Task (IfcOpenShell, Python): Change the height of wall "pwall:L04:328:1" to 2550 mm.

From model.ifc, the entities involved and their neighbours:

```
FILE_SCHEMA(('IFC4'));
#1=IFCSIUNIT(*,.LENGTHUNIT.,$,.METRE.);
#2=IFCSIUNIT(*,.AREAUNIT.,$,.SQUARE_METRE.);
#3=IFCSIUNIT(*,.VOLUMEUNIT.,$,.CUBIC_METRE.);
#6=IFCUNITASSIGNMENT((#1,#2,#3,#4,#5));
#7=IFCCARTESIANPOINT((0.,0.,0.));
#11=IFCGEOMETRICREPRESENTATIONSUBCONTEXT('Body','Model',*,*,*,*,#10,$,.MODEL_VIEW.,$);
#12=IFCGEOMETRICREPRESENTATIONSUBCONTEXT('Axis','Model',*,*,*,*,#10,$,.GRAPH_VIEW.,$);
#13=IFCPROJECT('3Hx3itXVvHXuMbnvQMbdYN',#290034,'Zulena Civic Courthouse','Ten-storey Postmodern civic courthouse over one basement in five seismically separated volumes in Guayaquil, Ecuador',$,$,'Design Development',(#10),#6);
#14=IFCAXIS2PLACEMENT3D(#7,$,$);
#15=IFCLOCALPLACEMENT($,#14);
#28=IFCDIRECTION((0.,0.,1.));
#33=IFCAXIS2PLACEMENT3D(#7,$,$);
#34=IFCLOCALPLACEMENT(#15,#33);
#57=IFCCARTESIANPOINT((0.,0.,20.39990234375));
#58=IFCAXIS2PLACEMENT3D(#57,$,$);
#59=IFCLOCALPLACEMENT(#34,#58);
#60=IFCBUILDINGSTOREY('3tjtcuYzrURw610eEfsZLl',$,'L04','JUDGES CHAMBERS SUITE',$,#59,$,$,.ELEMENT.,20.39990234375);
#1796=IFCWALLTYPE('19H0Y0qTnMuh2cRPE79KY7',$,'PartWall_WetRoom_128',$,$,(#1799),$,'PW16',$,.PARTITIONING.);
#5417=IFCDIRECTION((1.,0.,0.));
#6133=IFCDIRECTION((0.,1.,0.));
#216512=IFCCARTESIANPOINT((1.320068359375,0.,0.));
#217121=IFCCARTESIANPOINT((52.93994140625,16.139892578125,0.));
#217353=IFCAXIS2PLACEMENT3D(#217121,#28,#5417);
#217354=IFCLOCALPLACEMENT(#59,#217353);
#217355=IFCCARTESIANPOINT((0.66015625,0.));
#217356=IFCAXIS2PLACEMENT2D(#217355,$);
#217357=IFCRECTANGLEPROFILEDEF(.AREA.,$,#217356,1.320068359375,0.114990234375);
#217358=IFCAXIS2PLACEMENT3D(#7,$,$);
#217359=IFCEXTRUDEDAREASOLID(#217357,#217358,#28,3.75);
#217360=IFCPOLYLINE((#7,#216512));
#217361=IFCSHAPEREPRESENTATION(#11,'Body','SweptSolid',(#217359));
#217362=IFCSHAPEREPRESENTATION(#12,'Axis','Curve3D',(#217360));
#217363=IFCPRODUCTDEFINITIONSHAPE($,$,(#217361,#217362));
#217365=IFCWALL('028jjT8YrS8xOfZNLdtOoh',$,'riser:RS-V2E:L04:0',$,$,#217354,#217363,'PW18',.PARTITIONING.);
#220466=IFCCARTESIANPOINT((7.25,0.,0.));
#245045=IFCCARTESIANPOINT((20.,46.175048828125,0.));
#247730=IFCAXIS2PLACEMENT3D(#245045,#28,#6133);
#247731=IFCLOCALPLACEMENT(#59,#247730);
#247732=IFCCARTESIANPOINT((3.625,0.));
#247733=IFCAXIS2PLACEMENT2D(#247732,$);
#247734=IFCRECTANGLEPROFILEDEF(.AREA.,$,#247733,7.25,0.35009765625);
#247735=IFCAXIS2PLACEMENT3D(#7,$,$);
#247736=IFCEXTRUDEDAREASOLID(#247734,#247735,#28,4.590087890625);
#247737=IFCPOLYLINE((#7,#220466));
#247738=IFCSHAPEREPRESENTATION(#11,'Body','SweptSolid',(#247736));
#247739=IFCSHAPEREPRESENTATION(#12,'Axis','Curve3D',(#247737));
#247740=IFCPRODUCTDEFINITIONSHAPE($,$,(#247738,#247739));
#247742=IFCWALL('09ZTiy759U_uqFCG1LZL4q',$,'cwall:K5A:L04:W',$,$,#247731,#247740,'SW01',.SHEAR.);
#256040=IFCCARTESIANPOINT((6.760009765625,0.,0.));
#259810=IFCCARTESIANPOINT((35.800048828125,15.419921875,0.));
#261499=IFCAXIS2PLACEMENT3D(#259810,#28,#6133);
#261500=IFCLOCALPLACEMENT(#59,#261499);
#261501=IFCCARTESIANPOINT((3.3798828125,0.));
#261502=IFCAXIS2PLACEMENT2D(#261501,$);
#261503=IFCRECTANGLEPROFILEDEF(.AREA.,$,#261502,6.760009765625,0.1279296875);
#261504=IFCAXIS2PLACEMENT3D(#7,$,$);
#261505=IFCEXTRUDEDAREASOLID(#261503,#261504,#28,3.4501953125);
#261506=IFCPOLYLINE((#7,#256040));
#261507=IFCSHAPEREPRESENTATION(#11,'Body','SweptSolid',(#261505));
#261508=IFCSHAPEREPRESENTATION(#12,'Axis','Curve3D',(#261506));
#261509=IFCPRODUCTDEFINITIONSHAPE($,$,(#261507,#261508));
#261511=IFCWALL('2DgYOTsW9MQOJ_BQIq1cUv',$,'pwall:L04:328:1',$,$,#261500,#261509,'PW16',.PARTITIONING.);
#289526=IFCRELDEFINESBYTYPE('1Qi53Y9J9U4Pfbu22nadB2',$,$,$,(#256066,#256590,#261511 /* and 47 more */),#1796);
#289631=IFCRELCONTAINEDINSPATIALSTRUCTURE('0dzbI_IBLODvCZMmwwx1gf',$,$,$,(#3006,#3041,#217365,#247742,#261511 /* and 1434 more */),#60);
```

```python
import ifcopenshell
import ifcopenshell.geom
import ifcopenshell.util.representation
import ifcopenshell.util.shape
import ifcopenshell.util.unit

model = ifcopenshell.open("model.ifc")
unit_scale = ifcopenshell.util.unit.calculate_unit_scale(model)
settings = ifcopenshell.geom.settings()


def volume(element):
    """Net volume in cubic metres, openings subtracted."""
    shape = ifcopenshell.geom.create_shape(settings, element)
    return ifcopenshell.util.shape.get_volume(shape.geometry)


wall = model.by_guid("2DgYOTsW9MQOJ_BQIq1cUv")
before = volume(wall)

body = ifcopenshell.util.representation.get_representation(wall, "Model", "Body")
solid = body.Items[0]
old_height = solid.Depth
solid.Depth = 2.55 / unit_scale
after = volume(wall)

print(f"height {old_height:g} -> {solid.Depth:g}, volume {before:.3f} -> {after:.3f} m3")

model.write("model-out.ifc")
```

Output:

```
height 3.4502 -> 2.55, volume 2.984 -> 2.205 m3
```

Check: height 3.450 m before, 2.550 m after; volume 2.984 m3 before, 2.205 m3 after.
